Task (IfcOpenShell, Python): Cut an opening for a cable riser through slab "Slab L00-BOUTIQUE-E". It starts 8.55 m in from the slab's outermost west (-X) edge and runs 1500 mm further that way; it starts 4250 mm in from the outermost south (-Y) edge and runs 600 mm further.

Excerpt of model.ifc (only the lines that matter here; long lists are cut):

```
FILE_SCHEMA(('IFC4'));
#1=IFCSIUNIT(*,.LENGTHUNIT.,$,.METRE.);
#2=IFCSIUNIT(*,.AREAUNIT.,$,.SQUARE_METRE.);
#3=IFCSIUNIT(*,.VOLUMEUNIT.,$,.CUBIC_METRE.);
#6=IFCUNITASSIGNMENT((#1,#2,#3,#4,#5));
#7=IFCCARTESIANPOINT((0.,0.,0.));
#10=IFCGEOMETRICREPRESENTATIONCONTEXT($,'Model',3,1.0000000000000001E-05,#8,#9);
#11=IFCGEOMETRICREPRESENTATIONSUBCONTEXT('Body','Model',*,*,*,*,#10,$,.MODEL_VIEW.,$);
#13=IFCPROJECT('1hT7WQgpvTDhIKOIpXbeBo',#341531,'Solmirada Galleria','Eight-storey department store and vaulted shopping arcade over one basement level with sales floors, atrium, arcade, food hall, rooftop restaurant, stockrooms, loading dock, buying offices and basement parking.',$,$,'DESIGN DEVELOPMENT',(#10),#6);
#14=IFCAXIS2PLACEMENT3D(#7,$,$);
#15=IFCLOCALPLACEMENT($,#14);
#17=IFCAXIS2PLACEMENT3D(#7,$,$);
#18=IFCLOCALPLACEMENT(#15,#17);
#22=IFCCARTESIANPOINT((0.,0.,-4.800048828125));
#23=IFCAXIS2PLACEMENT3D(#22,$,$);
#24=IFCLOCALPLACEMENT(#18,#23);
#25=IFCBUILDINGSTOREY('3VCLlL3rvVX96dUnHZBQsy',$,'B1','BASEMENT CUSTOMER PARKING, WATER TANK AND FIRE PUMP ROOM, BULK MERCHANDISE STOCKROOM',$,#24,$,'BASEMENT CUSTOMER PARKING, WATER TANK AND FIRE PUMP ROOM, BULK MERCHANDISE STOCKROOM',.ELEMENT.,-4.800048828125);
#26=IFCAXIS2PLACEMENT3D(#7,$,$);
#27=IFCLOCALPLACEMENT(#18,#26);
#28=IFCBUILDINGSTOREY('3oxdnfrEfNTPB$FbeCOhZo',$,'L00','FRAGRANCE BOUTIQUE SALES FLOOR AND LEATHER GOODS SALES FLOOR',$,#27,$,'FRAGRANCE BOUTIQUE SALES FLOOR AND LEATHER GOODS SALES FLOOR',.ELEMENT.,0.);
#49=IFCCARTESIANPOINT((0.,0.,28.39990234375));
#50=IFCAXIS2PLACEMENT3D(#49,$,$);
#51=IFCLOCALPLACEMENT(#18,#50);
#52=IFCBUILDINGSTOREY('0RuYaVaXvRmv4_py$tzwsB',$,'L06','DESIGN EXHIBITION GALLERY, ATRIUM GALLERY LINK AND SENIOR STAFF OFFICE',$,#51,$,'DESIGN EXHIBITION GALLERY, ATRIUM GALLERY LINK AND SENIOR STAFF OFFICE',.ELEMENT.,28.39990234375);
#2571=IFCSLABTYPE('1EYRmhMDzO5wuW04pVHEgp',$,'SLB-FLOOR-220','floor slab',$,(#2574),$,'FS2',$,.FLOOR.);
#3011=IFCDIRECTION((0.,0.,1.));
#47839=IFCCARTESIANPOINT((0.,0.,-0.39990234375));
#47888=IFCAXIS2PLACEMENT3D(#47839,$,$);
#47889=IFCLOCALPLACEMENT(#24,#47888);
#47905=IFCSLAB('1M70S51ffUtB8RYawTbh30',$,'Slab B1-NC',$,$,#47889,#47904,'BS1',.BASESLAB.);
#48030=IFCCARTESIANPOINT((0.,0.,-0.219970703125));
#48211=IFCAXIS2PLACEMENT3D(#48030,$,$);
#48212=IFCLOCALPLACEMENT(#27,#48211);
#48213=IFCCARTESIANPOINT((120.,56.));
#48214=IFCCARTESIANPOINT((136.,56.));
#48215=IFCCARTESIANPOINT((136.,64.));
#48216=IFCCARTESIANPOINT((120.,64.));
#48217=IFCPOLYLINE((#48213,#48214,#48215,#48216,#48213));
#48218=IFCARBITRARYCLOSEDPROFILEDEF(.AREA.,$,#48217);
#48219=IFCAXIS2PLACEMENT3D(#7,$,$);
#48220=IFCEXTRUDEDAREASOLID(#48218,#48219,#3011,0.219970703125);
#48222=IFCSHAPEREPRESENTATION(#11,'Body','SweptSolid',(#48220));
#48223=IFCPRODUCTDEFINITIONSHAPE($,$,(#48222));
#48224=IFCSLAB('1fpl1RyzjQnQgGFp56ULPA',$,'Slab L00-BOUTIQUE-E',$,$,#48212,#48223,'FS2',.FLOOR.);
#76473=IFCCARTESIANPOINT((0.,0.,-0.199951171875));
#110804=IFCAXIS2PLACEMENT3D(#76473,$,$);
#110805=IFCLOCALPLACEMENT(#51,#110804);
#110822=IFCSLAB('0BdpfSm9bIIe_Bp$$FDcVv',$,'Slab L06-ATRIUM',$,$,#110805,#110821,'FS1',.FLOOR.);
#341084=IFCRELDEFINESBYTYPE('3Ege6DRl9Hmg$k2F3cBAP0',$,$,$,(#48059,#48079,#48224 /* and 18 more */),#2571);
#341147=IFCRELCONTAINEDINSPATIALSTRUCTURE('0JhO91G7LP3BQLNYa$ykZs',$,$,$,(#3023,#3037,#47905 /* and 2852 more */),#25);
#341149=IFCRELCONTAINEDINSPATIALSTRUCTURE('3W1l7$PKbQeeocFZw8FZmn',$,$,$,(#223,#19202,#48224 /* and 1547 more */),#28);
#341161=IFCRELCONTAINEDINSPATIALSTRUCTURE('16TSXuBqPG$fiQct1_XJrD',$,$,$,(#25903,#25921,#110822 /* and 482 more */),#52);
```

```python
import numpy as np
import ifcopenshell
import ifcopenshell.api.feature
import ifcopenshell.api.geometry
import ifcopenshell.api.root
import ifcopenshell.geom
import ifcopenshell.util.placement
import ifcopenshell.util.representation
import ifcopenshell.util.shape
import ifcopenshell.util.unit

model = ifcopenshell.open("model.ifc")
unit_scale = ifcopenshell.util.unit.calculate_unit_scale(model)
settings = ifcopenshell.geom.settings()


def volume(element):
    """Net volume in cubic metres, openings subtracted."""
    shape = ifcopenshell.geom.create_shape(settings, element)
    return ifcopenshell.util.shape.get_volume(shape.geometry)


slab = model.by_guid("1fpl1RyzjQnQgGFp56ULPA")
before = volume(slab)

# Extent in the slab's own axes, in metres. The edges named are its -X and -Y sides.
slab_shape = ifcopenshell.geom.create_shape(settings, slab)
vertices = ifcopenshell.util.shape.get_vertices(slab_shape.geometry)
x_min, y_min, bottom = vertices.min(axis=0)
top = vertices[:, 2].max()

opening = ifcopenshell.api.root.create_entity(model, ifc_class="IfcOpeningElement", name="Cable riser opening", predefined_type="OPENING")
context = ifcopenshell.util.representation.get_context(model, "Model", "Body", "MODEL_VIEW")
width, depth = 1.5, 0.6
outline = [(0.0, 0.0), (width, 0.0), (width, depth), (0.0, depth), (0.0, 0.0)]
# Overshoot both faces by 50 mm so the cut is clean.
shape = ifcopenshell.api.geometry.add_slab_representation(
    model, context=context, depth=top - bottom + 0.1, polyline=outline
)
ifcopenshell.api.geometry.assign_representation(model, product=opening, representation=shape)

matrix = ifcopenshell.util.placement.get_local_placement(slab.ObjectPlacement)
matrix[:, 3] = matrix @ np.append(np.array([x_min + 8.55, y_min + 4.25, bottom - 0.05]) / unit_scale, 1.0)
ifcopenshell.api.geometry.edit_object_placement(model, product=opening, matrix=matrix, is_si=False)
ifcopenshell.api.feature.add_feature(model, feature=opening, element=slab)

after = volume(slab)

print(f"slab volume {before:.3f} -> {after:.3f} m3")

model.write("model_updated.ifc")
```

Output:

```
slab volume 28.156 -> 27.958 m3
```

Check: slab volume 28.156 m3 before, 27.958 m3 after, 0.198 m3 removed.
